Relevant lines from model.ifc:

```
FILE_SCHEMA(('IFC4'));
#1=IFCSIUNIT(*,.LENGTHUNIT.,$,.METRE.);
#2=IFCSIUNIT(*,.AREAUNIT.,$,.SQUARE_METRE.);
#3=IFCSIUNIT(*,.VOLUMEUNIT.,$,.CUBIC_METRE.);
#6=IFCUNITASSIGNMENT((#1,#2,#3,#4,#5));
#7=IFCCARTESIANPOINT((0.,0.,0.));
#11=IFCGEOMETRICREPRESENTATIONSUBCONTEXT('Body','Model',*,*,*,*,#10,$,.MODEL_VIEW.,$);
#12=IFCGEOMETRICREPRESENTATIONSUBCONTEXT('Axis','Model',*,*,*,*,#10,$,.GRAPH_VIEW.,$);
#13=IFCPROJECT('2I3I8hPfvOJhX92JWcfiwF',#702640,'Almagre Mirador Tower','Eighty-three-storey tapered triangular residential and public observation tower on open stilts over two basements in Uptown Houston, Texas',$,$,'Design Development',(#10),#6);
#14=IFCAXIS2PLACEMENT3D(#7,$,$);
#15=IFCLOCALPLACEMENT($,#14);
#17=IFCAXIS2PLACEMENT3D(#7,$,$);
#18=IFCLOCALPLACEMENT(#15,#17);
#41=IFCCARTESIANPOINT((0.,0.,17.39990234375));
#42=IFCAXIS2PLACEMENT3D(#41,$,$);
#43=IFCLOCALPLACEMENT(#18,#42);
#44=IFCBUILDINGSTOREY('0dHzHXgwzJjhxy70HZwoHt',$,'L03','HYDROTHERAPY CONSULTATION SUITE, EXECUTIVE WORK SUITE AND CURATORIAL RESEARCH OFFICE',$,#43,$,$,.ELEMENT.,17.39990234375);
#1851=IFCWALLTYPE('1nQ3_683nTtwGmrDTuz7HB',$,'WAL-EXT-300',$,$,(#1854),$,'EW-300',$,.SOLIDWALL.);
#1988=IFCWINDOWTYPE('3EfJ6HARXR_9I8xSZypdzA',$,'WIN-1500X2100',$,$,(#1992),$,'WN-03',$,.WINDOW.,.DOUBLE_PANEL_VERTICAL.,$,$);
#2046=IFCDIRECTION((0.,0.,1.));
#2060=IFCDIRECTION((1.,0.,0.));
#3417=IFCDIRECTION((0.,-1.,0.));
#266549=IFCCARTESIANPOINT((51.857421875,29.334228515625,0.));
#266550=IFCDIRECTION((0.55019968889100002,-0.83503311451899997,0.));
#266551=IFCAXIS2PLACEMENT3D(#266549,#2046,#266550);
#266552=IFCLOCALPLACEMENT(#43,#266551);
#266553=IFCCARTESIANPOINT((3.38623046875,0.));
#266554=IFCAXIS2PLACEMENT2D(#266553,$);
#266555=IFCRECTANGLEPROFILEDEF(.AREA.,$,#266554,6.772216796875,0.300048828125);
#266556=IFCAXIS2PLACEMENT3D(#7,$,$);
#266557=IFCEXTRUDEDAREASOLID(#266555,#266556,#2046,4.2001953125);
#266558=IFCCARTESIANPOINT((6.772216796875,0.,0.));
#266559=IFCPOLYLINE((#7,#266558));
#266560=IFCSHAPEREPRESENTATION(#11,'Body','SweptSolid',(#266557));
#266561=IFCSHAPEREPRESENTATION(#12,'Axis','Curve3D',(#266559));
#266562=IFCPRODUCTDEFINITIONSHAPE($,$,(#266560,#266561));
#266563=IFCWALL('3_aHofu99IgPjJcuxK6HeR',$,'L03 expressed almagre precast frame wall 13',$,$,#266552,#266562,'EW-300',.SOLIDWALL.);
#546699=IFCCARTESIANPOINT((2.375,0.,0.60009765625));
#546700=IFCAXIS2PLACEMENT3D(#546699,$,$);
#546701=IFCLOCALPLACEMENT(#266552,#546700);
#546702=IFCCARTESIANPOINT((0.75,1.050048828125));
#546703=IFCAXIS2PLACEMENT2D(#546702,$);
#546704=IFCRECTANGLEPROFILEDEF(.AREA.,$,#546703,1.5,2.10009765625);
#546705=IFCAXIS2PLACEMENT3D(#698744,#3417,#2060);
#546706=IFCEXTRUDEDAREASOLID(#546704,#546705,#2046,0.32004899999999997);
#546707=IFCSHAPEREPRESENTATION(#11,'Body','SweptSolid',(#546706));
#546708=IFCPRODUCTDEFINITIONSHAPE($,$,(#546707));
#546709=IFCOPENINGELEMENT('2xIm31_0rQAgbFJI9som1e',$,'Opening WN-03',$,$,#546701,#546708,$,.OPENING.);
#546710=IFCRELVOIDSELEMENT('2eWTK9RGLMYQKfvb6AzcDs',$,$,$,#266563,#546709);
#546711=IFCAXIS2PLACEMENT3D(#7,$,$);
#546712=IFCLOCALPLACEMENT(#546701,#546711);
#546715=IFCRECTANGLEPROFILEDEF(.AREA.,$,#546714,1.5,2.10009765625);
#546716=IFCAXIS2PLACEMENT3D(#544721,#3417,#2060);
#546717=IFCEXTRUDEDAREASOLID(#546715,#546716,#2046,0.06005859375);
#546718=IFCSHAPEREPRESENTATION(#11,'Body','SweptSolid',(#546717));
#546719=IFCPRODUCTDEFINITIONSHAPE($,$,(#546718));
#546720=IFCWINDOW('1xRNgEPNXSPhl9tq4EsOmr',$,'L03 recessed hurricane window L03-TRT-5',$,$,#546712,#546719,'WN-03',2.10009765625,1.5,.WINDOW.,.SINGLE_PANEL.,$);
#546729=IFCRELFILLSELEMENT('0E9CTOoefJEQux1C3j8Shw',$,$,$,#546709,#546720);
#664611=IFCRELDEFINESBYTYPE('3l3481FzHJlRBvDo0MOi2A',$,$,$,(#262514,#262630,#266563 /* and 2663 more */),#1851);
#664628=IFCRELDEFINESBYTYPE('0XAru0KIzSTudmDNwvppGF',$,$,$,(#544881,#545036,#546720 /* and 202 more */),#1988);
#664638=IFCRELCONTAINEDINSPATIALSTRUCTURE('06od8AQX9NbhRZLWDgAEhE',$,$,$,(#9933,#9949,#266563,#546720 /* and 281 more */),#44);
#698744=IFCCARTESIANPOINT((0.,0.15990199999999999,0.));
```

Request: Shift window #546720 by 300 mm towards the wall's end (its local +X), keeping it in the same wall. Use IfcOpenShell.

```python
import ifcopenshell
import ifcopenshell.api.geometry
import ifcopenshell.util.placement
import ifcopenshell.util.unit

model = ifcopenshell.open("model.ifc")
unit_scale = ifcopenshell.util.unit.calculate_unit_scale(model)

window = model.by_guid("1xRNgEPNXSPhl9tq4EsOmr")
opening = window.FillsVoids[0].RelatingOpeningElement
wall = opening.VoidsElements[0].RelatingBuildingElement

wall_matrix = ifcopenshell.util.placement.get_local_placement(wall.ObjectPlacement)
shift = wall_matrix[:3, 0] * 0.3 / unit_scale
before = ifcopenshell.util.placement.get_local_placement(window.ObjectPlacement)[:3, 3].copy()

# The window is placed relative to its opening, so it follows when the opening moves.
matrix = ifcopenshell.util.placement.get_local_placement(opening.ObjectPlacement)
matrix[:3, 3] += shift
ifcopenshell.api.geometry.edit_object_placement(
    model, product=opening, matrix=matrix, is_si=False, should_transform_children=True
)

after = ifcopenshell.util.placement.get_local_placement(window.ObjectPlacement)[:3, 3]
print("window moved by", (after - before).round(3) + 0.0)

model.write("model-out.ifc")
```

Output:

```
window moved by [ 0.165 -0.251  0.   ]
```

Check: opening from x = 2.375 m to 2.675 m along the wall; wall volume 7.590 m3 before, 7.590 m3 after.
